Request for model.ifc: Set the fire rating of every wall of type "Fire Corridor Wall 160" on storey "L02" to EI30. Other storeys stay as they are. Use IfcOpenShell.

First a look at what the model holds.

```python
import ifcopenshell
import ifcopenshell.util.element

model = ifcopenshell.open("model.ifc")
print(model.schema)
storey = next(s for s in model.by_type("IfcBuildingStorey") if s.Name == "L02")
walls = [e for e in ifcopenshell.util.element.get_decomposition(storey) if e.is_a("IfcWall")]
seen = {}
for e in walls:
    element_type = ifcopenshell.util.element.get_type(e)
    key = (element_type.Name if element_type != e and element_type else None, ifcopenshell.util.element.get_pset(e, "Pset_WallCommon", "FireRating"))
    seen[key] = seen.get(key, 0) + 1
for (name, value), count in sorted(seen.items(), key=str):
    print(count, "x", name, "|", value)
```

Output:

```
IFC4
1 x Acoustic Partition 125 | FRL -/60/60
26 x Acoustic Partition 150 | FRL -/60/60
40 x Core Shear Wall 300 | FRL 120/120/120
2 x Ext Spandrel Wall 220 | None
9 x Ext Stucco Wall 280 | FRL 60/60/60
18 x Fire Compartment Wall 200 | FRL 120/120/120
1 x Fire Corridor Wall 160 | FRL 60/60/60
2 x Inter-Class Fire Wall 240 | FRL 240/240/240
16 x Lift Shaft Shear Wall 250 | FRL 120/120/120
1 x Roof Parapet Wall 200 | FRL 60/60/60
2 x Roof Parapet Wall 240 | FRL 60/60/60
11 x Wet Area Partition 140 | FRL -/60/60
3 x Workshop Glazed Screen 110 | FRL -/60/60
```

```python
import ifcopenshell
import ifcopenshell.api.pset
import ifcopenshell.util.element

model = ifcopenshell.open("model.ifc")

storey = next(s for s in model.by_type("IfcBuildingStorey") if s.Name == "L02")
walls = [e for e in ifcopenshell.util.element.get_decomposition(storey) if e.is_a("IfcWall")]

count = 0
for e in walls:
    element_type = ifcopenshell.util.element.get_type(e)
    if element_type in (None, e) or element_type.Name != "Fire Corridor Wall 160":
        continue
    # add_pset returns the element's existing set when there is one.
    pset = ifcopenshell.api.pset.add_pset(model, product=e, name="Pset_WallCommon")
    ifcopenshell.api.pset.edit_pset(model, pset=pset, properties={"FireRating": "EI30"})
    count += 1

print(count, "walls updated")

model.write("model_v2.ifc")
```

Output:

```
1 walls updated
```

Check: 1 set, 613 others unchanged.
